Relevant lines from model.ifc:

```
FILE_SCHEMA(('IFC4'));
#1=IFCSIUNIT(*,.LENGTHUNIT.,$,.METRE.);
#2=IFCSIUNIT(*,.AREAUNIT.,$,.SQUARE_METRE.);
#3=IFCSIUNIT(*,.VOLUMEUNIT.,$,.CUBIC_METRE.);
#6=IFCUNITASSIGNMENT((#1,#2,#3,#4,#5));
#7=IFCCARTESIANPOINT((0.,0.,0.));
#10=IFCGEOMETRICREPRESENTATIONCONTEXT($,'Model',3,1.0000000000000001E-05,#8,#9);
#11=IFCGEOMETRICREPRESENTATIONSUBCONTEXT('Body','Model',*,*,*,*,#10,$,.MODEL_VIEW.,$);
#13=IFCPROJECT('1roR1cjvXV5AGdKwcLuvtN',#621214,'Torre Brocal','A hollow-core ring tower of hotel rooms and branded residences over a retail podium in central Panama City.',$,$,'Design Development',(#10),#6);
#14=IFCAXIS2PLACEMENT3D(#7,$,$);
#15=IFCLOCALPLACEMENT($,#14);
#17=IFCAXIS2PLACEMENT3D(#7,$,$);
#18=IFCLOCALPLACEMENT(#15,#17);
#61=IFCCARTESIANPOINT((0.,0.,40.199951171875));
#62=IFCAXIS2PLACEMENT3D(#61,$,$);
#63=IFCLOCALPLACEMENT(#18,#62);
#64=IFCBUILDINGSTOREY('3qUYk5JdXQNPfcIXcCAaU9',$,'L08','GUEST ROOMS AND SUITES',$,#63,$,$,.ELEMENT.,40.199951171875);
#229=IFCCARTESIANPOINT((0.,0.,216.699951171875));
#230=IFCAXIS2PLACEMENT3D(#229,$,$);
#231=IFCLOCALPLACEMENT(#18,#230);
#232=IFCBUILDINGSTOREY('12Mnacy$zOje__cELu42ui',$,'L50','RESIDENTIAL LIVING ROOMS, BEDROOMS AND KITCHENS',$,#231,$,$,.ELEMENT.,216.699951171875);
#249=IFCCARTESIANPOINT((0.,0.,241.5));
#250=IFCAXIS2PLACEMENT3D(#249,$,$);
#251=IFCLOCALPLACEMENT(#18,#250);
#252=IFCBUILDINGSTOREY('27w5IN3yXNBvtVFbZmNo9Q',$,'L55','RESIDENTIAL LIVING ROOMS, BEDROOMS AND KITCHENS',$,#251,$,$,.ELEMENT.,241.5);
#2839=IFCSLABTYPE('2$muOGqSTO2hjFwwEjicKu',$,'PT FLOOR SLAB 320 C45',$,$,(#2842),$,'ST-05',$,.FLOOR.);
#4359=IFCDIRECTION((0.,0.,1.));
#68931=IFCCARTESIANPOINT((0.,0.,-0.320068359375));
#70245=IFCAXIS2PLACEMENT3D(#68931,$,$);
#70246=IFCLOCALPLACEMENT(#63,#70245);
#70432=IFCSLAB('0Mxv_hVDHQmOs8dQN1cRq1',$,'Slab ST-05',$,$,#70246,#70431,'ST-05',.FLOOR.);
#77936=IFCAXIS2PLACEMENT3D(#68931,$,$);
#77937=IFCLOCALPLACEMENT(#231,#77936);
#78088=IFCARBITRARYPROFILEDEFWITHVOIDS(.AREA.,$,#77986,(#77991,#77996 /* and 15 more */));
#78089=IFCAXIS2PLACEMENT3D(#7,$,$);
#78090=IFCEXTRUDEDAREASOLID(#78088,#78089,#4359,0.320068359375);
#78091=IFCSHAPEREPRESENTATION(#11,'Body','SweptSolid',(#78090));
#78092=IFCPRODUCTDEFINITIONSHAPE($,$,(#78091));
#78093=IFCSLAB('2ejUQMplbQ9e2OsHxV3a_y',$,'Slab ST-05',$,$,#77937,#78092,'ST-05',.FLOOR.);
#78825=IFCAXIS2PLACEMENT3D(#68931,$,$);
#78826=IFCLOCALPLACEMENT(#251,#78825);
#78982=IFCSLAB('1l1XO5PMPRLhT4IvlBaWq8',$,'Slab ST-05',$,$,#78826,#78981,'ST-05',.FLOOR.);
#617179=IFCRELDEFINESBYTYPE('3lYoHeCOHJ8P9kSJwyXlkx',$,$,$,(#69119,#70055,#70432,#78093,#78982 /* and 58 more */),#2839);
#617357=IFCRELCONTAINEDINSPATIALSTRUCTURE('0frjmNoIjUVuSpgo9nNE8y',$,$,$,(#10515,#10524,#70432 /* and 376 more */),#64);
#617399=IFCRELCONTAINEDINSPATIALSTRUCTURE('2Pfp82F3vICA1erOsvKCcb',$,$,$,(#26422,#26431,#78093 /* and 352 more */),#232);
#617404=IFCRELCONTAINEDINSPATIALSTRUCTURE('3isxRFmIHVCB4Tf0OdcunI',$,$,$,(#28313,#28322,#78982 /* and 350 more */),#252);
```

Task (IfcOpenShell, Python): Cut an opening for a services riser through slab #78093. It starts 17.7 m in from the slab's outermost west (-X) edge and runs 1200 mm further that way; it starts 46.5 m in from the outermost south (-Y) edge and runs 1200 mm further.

```python
import numpy as np
import ifcopenshell
import ifcopenshell.api.feature
import ifcopenshell.api.geometry
import ifcopenshell.api.root
import ifcopenshell.geom
import ifcopenshell.util.placement
import ifcopenshell.util.representation
import ifcopenshell.util.shape
import ifcopenshell.util.unit

model = ifcopenshell.open("model.ifc")
unit_scale = ifcopenshell.util.unit.calculate_unit_scale(model)
settings = ifcopenshell.geom.settings()


def volume(element):
    """Net volume in cubic metres, openings subtracted."""
    shape = ifcopenshell.geom.create_shape(settings, element)
    return ifcopenshell.util.shape.get_volume(shape.geometry)


slab = model.by_guid("2ejUQMplbQ9e2OsHxV3a_y")
before = volume(slab)

# Extent in the slab's own axes, in metres. The edges named are its -X and -Y sides.
slab_shape = ifcopenshell.geom.create_shape(settings, slab)
vertices = ifcopenshell.util.shape.get_vertices(slab_shape.geometry)
x_min, y_min, bottom = vertices.min(axis=0)
top = vertices[:, 2].max()

opening = ifcopenshell.api.root.create_entity(model, ifc_class="IfcOpeningElement", name="Services riser opening", predefined_type="OPENING")
context = ifcopenshell.util.representation.get_context(model, "Model", "Body", "MODEL_VIEW")
width, depth = 1.2, 1.2
outline = [(0.0, 0.0), (width, 0.0), (width, depth), (0.0, depth), (0.0, 0.0)]
# Overshoot both faces by 50 mm so the cut is clean.
shape = ifcopenshell.api.geometry.add_slab_representation(
    model, context=context, depth=top - bottom + 0.1, polyline=outline
)
ifcopenshell.api.geometry.assign_representation(model, product=opening, representation=shape)

matrix = ifcopenshell.util.placement.get_local_placement(slab.ObjectPlacement)
matrix[:, 3] = matrix @ np.append(np.array([x_min + 17.7, y_min + 46.5, bottom - 0.05]) / unit_scale, 1.0)
ifcopenshell.api.geometry.edit_object_placement(model, product=opening, matrix=matrix, is_si=False)
ifcopenshell.api.feature.add_feature(model, feature=opening, element=slab)

after = volume(slab)

print(f"slab volume {before:.3f} -> {after:.3f} m3")

model.write("model_rev.ifc")
```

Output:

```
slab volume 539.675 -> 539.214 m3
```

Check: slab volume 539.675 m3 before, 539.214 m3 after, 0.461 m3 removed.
